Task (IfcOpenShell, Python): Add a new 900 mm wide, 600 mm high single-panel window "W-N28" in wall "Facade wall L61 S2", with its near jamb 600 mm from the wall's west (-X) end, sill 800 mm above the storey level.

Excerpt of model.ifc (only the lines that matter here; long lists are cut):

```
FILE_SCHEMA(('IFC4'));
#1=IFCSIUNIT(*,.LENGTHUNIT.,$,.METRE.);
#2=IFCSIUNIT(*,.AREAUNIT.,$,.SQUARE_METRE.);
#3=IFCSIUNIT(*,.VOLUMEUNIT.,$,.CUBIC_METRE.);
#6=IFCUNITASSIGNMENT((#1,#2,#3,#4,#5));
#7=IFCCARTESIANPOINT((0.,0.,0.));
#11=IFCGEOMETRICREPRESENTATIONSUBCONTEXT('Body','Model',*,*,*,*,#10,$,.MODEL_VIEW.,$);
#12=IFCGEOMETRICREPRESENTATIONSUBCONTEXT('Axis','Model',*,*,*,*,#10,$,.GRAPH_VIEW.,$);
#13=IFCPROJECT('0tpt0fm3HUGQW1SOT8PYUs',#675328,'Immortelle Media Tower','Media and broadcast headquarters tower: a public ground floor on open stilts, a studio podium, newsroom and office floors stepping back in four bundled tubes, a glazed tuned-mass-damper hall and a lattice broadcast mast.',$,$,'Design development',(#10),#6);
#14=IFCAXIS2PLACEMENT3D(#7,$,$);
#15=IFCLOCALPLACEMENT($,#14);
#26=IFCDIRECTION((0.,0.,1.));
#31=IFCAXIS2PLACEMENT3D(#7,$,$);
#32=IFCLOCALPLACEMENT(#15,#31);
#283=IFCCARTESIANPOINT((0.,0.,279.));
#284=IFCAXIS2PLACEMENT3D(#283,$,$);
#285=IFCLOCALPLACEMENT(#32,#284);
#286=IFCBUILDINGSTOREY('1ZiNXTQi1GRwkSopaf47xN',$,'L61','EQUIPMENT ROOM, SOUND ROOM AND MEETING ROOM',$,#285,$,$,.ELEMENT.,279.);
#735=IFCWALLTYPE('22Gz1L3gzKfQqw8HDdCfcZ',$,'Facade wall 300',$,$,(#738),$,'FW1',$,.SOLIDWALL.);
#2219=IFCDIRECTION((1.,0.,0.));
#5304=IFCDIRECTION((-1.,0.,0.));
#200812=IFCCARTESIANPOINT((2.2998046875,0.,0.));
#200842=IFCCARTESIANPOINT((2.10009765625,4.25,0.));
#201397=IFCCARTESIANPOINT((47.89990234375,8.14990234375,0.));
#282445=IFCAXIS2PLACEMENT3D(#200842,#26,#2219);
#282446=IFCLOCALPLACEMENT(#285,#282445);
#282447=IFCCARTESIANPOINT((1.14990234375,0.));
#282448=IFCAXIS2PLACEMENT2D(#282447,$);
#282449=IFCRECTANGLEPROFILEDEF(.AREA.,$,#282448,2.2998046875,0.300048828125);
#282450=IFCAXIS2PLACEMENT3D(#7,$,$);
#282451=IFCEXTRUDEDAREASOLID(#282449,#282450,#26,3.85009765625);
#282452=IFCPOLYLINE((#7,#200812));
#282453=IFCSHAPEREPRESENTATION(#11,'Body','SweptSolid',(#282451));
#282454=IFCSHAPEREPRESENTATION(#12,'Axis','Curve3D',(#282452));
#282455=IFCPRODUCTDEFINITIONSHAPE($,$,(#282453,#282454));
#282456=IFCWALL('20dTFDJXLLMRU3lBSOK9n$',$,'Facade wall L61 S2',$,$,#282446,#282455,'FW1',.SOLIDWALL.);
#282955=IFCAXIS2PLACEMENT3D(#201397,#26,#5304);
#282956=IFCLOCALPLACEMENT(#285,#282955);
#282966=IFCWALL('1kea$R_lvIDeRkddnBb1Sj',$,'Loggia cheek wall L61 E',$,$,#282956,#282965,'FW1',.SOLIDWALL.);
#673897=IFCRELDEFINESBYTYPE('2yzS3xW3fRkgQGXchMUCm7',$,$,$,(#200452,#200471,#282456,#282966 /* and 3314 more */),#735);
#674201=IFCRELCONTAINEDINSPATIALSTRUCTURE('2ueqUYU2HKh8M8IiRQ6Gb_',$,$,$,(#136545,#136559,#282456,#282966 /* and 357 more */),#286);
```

```python
import numpy as np
import ifcopenshell
import ifcopenshell.api.feature
import ifcopenshell.api.geometry
import ifcopenshell.api.root
import ifcopenshell.api.spatial
import ifcopenshell.geom
import ifcopenshell.util.element
import ifcopenshell.util.placement
import ifcopenshell.util.representation
import ifcopenshell.util.shape
import ifcopenshell.util.unit

model = ifcopenshell.open("model.ifc")
unit_scale = ifcopenshell.util.unit.calculate_unit_scale(model)
settings = ifcopenshell.geom.settings()


def volume(element):
    """Net volume in cubic metres, openings subtracted."""
    shape = ifcopenshell.geom.create_shape(settings, element)
    return ifcopenshell.util.shape.get_volume(shape.geometry)


wall = model.by_guid("20dTFDJXLLMRU3lBSOK9n$")
storey = ifcopenshell.util.element.get_container(wall, ifc_class="IfcBuildingStorey")
context = ifcopenshell.util.representation.get_context(model, "Model", "Body", "MODEL_VIEW")
before = volume(wall)

width, height, from_end, sill = 0.9, 0.6, 0.6, 0.8  # metres

# The wall runs along its own X axis, and the end named is its -X end.
wall_shape = ifcopenshell.geom.create_shape(settings, wall)
x, y, z = ifcopenshell.util.shape.get_vertices(wall_shape.geometry).T
start = x.min() + from_end
face, thickness = float(y.min()), float(y.max() - y.min())
wall_matrix = ifcopenshell.util.placement.get_local_placement(wall.ObjectPlacement)
level = ifcopenshell.util.placement.get_local_placement(storey.ObjectPlacement)[2, 3]


def in_wall(x, y):
    """Placement at x, y metres in the wall's axes, at sill height."""
    matrix = wall_matrix.copy()
    matrix[:, 3] = wall_matrix @ np.array([x / unit_scale, y / unit_scale, 0.0, 1.0])
    matrix[2, 3] = level + sill / unit_scale
    return matrix


# Opening: a box that overshoots both wall faces by 50 mm.
opening = ifcopenshell.api.root.create_entity(model, ifc_class="IfcOpeningElement", predefined_type="OPENING")
box = ifcopenshell.api.geometry.add_wall_representation(
    model, context=context, length=width, height=height, thickness=thickness + 0.1
)
ifcopenshell.api.geometry.assign_representation(model, product=opening, representation=box)
ifcopenshell.api.geometry.edit_object_placement(model, product=opening, matrix=in_wall(start, face - 0.05), is_si=False)
ifcopenshell.api.feature.add_feature(model, feature=opening, element=wall)

window = ifcopenshell.api.root.create_entity(model, ifc_class="IfcWindow", name="W-N28", predefined_type="WINDOW")
window.OverallWidth, window.OverallHeight = width / unit_scale, height / unit_scale
window.PartitioningType = "SINGLE_PANEL"
body = ifcopenshell.api.geometry.add_window_representation(
    model,
    context=context,
    overall_width=window.OverallWidth,
    overall_height=window.OverallHeight,
    partition_type="SINGLE_PANEL",
)
ifcopenshell.api.geometry.assign_representation(model, product=window, representation=body)
ifcopenshell.api.spatial.assign_container(model, products=[window], relating_structure=storey)
ifcopenshell.api.feature.add_filling(model, opening=opening, element=window)

# Centre the window in the wall's thickness.
ifcopenshell.api.geometry.edit_object_placement(model, product=window, matrix=in_wall(start, face), is_si=False)
window_shape = ifcopenshell.geom.create_shape(settings, window)
depth = ifcopenshell.util.shape.get_vertices(window_shape.geometry)[:, 1]
offset = face + thickness / 2 - (depth.min() + depth.max()) / 2
ifcopenshell.api.geometry.edit_object_placement(model, product=window, matrix=in_wall(start, offset), is_si=False)

after = volume(wall)

print(f"wall volume {before:.3f} -> {after:.3f} m3")

model.write("model-out.ifc")
```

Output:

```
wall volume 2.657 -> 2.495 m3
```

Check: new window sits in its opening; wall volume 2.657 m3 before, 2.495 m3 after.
